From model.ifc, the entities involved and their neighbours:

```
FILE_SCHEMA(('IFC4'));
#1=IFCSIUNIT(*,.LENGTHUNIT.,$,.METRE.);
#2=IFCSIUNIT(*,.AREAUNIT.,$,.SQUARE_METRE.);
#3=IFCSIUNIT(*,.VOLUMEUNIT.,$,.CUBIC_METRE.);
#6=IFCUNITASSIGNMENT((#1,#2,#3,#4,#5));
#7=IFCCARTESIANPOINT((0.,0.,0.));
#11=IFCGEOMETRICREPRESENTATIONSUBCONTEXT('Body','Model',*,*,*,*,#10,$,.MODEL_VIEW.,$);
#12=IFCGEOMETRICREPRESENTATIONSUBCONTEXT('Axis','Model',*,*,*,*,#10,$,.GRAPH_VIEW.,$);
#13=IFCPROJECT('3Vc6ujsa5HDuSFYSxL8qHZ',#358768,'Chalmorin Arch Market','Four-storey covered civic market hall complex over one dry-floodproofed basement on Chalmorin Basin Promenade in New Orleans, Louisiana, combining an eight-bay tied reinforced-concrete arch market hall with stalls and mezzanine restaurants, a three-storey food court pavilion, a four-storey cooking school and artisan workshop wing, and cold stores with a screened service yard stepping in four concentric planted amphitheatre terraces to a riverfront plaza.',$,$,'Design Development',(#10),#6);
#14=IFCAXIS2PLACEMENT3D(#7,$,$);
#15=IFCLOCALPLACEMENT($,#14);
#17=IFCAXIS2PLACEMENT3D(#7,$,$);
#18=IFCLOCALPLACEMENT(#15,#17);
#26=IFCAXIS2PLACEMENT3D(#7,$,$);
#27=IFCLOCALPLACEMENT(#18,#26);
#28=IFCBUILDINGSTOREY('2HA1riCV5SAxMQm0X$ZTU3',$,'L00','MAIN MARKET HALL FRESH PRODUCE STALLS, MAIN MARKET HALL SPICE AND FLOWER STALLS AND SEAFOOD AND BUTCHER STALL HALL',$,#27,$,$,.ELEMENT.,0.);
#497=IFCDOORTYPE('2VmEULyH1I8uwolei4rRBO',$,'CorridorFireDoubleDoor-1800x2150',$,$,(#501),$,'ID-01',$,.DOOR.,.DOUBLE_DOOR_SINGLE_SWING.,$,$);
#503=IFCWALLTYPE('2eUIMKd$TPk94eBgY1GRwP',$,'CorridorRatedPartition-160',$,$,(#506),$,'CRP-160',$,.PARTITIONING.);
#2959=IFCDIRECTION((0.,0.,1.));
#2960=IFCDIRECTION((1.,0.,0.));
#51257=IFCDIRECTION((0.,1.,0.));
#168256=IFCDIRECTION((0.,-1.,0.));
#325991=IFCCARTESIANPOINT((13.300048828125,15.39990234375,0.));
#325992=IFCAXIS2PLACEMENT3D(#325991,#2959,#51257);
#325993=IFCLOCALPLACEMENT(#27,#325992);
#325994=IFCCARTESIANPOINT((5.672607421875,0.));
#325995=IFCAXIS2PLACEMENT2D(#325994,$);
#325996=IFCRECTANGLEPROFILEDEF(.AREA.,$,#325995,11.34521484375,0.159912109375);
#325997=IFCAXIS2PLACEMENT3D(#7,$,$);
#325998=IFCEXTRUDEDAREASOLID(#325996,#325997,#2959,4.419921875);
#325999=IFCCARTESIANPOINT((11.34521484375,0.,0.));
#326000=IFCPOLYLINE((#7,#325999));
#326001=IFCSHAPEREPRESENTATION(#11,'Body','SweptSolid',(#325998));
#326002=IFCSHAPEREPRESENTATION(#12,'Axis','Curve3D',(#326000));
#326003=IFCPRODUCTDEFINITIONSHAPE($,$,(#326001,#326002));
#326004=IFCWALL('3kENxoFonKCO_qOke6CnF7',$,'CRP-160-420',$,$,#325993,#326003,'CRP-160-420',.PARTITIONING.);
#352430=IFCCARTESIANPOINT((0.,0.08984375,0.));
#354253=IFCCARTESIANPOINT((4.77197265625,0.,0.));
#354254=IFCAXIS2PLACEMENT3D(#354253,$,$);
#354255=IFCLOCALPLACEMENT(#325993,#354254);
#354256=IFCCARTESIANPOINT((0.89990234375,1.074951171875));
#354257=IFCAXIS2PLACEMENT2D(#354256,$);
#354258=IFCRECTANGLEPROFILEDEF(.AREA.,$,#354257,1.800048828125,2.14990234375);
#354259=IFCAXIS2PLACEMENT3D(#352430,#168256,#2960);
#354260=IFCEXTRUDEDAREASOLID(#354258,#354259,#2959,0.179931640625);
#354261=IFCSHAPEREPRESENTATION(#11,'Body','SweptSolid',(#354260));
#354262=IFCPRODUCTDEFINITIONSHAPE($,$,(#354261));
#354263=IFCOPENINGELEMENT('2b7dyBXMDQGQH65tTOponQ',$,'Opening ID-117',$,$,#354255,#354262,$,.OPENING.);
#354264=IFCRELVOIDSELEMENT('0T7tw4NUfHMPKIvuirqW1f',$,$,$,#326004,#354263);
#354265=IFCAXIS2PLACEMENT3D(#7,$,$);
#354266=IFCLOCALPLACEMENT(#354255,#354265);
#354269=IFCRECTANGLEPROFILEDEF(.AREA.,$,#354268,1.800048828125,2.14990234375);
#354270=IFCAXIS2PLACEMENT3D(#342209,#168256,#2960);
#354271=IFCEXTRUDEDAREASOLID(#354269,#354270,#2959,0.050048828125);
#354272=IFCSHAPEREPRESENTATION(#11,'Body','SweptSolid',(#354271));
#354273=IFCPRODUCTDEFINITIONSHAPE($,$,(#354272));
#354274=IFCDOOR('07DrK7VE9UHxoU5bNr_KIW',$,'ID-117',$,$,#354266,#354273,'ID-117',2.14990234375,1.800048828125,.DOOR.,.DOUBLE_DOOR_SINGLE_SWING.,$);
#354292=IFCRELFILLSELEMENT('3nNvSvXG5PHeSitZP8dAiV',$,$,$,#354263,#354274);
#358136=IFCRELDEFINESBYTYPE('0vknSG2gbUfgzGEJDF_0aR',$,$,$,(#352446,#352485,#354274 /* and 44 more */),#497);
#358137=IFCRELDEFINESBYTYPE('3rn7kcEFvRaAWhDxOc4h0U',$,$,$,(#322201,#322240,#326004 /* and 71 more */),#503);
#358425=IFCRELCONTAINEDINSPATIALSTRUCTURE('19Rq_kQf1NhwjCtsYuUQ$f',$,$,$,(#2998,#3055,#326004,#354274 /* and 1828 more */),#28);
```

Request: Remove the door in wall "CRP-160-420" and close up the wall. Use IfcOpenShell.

```python
import ifcopenshell
import ifcopenshell.api.feature
import ifcopenshell.api.root
import ifcopenshell.geom
import ifcopenshell.util.shape

model = ifcopenshell.open("model.ifc")
settings = ifcopenshell.geom.settings()


def volume(element):
    """Net volume in cubic metres, openings subtracted."""
    shape = ifcopenshell.geom.create_shape(settings, element)
    return ifcopenshell.util.shape.get_volume(shape.geometry)


door = model.by_guid("07DrK7VE9UHxoU5bNr_KIW")
opening = door.FillsVoids[0].RelatingOpeningElement
wall = opening.VoidsElements[0].RelatingBuildingElement
before = volume(wall)

ifcopenshell.api.root.remove_product(model, product=door)
ifcopenshell.api.feature.remove_feature(model, feature=opening)

after = volume(wall)

print(f"wall volume {before:.3f} -> {after:.3f} m3")

model.write("model_rev.ifc")
```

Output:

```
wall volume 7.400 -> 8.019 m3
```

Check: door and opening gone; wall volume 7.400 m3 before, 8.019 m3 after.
